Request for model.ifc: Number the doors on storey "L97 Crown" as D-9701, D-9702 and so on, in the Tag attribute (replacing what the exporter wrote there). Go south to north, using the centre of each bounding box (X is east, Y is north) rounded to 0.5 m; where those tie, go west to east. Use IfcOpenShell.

First a look at what the model holds.

```python
import ifcopenshell
import ifcopenshell.util.element
import ifcopenshell.util.placement

model = ifcopenshell.open("model.ifc")
print(model.schema)
storey = next(s for s in model.by_type("IfcBuildingStorey") if s.Name == "L97 Crown")
doors = [e for e in ifcopenshell.util.element.get_decomposition(storey) if e.is_a("IfcDoor")]
for e in sorted(doors, key=lambda e: e.id()):
    origin = ifcopenshell.util.placement.get_local_placement(e.ObjectPlacement)[:3, 3]
    print(e.id(), e.Tag, e.Name, origin.round(2) + 0.0, sep=" | ")
```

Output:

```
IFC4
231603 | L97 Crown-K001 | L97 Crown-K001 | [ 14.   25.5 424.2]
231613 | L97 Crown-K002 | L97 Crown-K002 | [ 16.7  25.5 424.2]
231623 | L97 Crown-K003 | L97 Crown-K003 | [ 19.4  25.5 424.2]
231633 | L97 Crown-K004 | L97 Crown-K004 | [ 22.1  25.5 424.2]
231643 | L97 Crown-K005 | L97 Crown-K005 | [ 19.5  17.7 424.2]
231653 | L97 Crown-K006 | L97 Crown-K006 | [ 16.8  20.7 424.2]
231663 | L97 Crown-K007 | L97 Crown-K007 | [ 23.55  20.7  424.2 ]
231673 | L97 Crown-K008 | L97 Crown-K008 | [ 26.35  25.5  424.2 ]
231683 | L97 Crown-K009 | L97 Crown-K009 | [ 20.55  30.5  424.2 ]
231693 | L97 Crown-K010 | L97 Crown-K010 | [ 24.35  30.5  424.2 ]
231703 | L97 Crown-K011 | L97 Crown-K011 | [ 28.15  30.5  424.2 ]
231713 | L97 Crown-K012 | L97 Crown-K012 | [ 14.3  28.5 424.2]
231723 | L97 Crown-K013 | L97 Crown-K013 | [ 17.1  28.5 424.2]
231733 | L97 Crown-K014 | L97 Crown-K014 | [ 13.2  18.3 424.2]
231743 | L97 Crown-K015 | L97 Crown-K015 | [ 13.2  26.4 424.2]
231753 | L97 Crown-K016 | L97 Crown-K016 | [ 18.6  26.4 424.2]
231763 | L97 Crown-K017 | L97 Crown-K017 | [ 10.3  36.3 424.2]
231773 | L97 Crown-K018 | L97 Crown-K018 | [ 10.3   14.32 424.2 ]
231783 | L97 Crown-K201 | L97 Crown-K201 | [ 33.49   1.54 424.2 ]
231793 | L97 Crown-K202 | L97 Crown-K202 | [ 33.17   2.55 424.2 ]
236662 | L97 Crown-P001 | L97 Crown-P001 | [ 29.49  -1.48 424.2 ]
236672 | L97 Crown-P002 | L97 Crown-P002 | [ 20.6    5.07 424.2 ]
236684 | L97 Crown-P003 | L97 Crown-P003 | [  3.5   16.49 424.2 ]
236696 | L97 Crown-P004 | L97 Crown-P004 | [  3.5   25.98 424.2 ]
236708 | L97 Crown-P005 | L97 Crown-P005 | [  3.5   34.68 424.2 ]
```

```python
import ifcopenshell
import ifcopenshell.geom
import ifcopenshell.util.element
import ifcopenshell.util.shape

model = ifcopenshell.open("model.ifc")
settings = ifcopenshell.geom.settings()
settings.set("use-world-coords", True)


def centre(element):
    shape = ifcopenshell.geom.create_shape(settings, element)
    return ifcopenshell.util.shape.get_bbox_centroid(shape.geometry)


storey = next(s for s in model.by_type("IfcBuildingStorey") if s.Name == "L97 Crown")
doors = [e for e in ifcopenshell.util.element.get_decomposition(storey) if e.is_a("IfcDoor")]

# Insertion points can sit at a corner or the storey origin, so sort by the geometry (in metres).
centres = {e: centre(e) for e in doors}
doors.sort(key=lambda e: (round(centres[e][1] / 0.5), centres[e][0]))

for i, e in enumerate(doors, start=1):
    number = f"D-97{i:02d}"
    e.Tag = number
    print(e.id(), number)

model.write("model-out.ifc")
```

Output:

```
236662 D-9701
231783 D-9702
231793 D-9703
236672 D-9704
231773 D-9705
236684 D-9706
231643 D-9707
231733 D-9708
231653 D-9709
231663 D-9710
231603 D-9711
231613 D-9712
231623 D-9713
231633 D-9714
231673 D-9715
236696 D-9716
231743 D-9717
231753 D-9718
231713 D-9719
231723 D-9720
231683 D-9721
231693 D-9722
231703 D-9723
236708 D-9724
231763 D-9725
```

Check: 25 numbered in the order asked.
